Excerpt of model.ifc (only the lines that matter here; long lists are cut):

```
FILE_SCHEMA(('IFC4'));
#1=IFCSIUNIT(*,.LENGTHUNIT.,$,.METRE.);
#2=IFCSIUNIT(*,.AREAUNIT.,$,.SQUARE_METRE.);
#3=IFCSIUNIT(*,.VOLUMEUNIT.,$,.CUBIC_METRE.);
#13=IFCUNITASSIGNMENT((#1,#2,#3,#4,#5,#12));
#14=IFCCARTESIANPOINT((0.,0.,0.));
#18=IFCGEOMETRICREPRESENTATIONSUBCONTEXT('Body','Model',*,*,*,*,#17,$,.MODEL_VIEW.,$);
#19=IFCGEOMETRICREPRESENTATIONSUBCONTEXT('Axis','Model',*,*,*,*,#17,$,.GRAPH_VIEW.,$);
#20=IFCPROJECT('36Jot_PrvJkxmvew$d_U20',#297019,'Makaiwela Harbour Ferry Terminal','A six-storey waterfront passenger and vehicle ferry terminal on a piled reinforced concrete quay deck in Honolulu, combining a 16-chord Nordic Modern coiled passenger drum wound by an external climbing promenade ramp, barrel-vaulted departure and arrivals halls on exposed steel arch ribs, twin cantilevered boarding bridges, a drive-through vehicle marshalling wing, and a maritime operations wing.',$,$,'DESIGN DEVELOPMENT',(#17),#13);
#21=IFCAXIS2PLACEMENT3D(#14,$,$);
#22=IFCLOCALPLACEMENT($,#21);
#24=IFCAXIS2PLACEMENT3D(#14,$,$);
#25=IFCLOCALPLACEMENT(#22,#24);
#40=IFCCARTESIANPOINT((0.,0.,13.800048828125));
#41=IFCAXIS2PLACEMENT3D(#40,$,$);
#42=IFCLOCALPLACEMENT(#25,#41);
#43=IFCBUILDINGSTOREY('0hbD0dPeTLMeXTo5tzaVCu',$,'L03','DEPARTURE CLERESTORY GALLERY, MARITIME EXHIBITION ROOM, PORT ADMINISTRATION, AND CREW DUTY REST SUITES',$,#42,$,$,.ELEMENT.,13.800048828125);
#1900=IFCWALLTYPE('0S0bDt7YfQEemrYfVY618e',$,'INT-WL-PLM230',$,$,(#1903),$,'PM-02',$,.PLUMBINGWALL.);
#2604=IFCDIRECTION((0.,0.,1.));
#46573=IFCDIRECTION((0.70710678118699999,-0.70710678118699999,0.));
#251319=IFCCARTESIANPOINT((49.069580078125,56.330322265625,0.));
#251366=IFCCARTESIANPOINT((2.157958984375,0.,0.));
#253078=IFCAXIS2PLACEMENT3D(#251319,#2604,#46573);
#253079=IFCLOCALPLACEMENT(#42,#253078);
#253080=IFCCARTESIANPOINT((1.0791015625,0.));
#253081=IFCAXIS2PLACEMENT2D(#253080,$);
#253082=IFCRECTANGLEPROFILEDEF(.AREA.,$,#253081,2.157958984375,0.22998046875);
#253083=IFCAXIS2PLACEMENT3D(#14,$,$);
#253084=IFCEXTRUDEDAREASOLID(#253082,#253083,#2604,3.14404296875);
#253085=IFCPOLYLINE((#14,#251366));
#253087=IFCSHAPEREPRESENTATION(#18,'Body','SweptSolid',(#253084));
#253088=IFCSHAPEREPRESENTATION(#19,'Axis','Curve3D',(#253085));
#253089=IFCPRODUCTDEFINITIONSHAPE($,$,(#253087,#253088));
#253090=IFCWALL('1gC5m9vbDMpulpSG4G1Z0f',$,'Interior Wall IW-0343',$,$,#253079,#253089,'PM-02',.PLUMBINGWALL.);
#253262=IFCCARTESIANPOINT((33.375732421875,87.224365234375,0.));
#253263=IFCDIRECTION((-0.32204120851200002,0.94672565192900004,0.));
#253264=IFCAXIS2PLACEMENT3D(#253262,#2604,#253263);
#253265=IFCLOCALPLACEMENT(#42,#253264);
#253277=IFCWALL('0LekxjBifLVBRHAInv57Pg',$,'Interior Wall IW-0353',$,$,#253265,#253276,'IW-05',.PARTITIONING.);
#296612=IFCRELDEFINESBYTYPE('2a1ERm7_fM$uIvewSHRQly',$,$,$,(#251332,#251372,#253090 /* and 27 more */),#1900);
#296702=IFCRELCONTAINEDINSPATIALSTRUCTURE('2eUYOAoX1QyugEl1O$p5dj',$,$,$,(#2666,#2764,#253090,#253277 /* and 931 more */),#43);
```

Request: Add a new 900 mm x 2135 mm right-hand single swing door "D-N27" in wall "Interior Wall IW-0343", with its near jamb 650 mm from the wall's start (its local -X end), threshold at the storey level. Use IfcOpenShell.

```python
import numpy as np
import ifcopenshell
import ifcopenshell.api.feature
import ifcopenshell.api.geometry
import ifcopenshell.api.root
import ifcopenshell.api.spatial
import ifcopenshell.geom
import ifcopenshell.util.element
import ifcopenshell.util.placement
import ifcopenshell.util.representation
import ifcopenshell.util.shape
import ifcopenshell.util.unit

model = ifcopenshell.open("model.ifc")
unit_scale = ifcopenshell.util.unit.calculate_unit_scale(model)
settings = ifcopenshell.geom.settings()


def volume(element):
    """Net volume in cubic metres, openings subtracted."""
    shape = ifcopenshell.geom.create_shape(settings, element)
    return ifcopenshell.util.shape.get_volume(shape.geometry)


wall = model.by_guid("1gC5m9vbDMpulpSG4G1Z0f")
storey = ifcopenshell.util.element.get_container(wall, ifc_class="IfcBuildingStorey")
context = ifcopenshell.util.representation.get_context(model, "Model", "Body", "MODEL_VIEW")
before = volume(wall)

width, height, from_end, sill = 0.9, 2.135, 0.65, 0.0  # metres

# The wall runs along its own X axis, and the end named is its -X end.
wall_shape = ifcopenshell.geom.create_shape(settings, wall)
x, y, z = ifcopenshell.util.shape.get_vertices(wall_shape.geometry).T
start = x.min() + from_end
face, thickness = float(y.min()), float(y.max() - y.min())
wall_matrix = ifcopenshell.util.placement.get_local_placement(wall.ObjectPlacement)
level = ifcopenshell.util.placement.get_local_placement(storey.ObjectPlacement)[2, 3]


def in_wall(x, y):
    """Placement at x, y metres in the wall's axes, at sill height."""
    matrix = wall_matrix.copy()
    matrix[:, 3] = wall_matrix @ np.array([x / unit_scale, y / unit_scale, 0.0, 1.0])
    matrix[2, 3] = level + sill / unit_scale
    return matrix


# Opening: a box that overshoots both wall faces by 50 mm.
opening = ifcopenshell.api.root.create_entity(model, ifc_class="IfcOpeningElement", predefined_type="OPENING")
box = ifcopenshell.api.geometry.add_wall_representation(
    model, context=context, length=width, height=height, thickness=thickness + 0.1
)
ifcopenshell.api.geometry.assign_representation(model, product=opening, representation=box)
ifcopenshell.api.geometry.edit_object_placement(model, product=opening, matrix=in_wall(start, face - 0.05), is_si=False)
ifcopenshell.api.feature.add_feature(model, feature=opening, element=wall)

door = ifcopenshell.api.root.create_entity(model, ifc_class="IfcDoor", name="D-N27", predefined_type="DOOR")
door.OverallWidth, door.OverallHeight = width / unit_scale, height / unit_scale
door.OperationType = "SINGLE_SWING_RIGHT"
body = ifcopenshell.api.geometry.add_door_representation(
    model,
    context=context,
    overall_width=door.OverallWidth,
    overall_height=door.OverallHeight,
    operation_type="SINGLE_SWING_RIGHT",
    lining_properties={"LiningDepth": thickness / unit_scale, "ThresholdDepth": thickness / unit_scale},
)
ifcopenshell.api.geometry.assign_representation(model, product=door, representation=body)
ifcopenshell.api.spatial.assign_container(model, products=[door], relating_structure=storey)
ifcopenshell.api.feature.add_filling(model, opening=opening, element=door)

# The lining spans the wall, so the door starts at the wall face.
ifcopenshell.api.geometry.edit_object_placement(model, product=door, matrix=in_wall(start, face), is_si=False)

after = volume(wall)

print(f"wall volume {before:.3f} -> {after:.3f} m3")

model.write("model_updated.ifc")
```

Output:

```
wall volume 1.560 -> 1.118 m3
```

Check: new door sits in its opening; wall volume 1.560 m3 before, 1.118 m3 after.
